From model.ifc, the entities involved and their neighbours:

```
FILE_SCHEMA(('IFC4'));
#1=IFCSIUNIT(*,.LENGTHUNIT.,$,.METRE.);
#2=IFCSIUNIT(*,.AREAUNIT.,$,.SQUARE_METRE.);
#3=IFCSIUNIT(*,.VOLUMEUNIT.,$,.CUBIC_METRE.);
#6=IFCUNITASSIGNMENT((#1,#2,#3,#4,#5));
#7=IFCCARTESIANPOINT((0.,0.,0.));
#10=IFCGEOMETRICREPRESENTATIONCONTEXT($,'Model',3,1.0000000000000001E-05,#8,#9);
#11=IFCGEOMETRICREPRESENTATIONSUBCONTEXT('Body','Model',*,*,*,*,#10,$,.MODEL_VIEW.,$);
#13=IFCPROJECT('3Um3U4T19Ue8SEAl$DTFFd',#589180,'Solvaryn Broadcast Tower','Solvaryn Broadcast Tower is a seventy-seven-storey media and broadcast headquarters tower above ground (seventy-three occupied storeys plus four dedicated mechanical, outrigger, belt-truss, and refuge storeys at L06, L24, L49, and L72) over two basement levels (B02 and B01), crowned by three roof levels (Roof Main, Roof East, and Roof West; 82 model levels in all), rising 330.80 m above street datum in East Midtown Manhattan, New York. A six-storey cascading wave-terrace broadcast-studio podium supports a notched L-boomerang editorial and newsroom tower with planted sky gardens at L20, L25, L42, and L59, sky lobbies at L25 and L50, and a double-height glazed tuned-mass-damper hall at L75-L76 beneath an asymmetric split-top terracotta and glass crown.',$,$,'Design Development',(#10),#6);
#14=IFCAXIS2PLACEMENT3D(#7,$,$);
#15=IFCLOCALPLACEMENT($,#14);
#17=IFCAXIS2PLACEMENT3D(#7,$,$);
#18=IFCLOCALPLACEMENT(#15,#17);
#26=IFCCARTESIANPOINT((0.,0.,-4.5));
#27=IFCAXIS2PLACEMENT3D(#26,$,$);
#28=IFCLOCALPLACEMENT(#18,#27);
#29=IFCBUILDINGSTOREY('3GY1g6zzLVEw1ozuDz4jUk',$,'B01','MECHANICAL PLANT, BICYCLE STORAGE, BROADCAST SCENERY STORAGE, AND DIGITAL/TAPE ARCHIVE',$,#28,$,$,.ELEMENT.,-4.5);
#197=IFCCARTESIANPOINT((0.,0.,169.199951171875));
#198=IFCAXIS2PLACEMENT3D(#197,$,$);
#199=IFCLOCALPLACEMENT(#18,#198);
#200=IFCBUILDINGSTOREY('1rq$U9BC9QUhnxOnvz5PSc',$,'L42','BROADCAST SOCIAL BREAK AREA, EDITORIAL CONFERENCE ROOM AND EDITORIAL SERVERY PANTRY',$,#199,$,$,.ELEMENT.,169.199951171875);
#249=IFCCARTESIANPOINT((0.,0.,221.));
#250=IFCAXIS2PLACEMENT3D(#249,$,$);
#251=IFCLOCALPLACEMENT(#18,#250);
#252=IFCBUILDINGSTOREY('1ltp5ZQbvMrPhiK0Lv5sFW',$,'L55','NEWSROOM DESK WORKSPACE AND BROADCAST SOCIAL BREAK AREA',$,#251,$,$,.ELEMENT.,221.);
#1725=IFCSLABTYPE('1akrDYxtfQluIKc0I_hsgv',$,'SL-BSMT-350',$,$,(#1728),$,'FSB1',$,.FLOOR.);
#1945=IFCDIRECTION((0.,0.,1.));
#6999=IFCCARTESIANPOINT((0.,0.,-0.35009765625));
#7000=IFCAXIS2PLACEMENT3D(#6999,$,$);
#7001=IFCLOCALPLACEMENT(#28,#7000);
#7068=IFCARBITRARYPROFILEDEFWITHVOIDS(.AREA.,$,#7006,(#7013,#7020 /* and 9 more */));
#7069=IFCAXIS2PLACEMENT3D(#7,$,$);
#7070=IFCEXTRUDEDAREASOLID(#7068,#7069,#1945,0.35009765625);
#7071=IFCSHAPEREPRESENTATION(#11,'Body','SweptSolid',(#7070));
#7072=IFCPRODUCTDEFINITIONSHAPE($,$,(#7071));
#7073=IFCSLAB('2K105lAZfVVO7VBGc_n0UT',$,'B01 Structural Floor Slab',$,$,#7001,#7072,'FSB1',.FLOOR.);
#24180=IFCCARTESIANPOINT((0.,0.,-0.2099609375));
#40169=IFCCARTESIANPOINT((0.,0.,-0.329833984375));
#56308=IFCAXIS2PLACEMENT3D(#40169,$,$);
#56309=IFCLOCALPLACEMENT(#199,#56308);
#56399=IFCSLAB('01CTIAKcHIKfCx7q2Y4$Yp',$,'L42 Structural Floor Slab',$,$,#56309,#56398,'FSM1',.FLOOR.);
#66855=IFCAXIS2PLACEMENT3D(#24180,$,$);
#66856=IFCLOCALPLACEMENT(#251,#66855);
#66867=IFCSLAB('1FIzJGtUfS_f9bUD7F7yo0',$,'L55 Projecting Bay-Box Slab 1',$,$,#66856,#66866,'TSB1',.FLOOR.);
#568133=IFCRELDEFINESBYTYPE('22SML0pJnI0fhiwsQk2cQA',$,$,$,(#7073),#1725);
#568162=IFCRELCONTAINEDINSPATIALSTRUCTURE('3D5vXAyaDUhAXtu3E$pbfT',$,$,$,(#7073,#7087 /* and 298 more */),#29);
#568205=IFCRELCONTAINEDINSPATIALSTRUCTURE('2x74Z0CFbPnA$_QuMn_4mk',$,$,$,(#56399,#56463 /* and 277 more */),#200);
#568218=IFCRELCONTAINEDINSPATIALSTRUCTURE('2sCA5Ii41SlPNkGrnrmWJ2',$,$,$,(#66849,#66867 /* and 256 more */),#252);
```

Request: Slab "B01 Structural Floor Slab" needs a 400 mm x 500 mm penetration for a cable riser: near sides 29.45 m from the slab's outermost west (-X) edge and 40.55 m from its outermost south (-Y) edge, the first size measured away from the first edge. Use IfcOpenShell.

```python
import numpy as np
import ifcopenshell
import ifcopenshell.api.feature
import ifcopenshell.api.geometry
import ifcopenshell.api.root
import ifcopenshell.geom
import ifcopenshell.util.placement
import ifcopenshell.util.representation
import ifcopenshell.util.shape
import ifcopenshell.util.unit

model = ifcopenshell.open("model.ifc")
unit_scale = ifcopenshell.util.unit.calculate_unit_scale(model)
settings = ifcopenshell.geom.settings()


def volume(element):
    """Net volume in cubic metres, openings subtracted."""
    shape = ifcopenshell.geom.create_shape(settings, element)
    return ifcopenshell.util.shape.get_volume(shape.geometry)


slab = model.by_guid("2K105lAZfVVO7VBGc_n0UT")
before = volume(slab)

# Extent in the slab's own axes, in metres. The edges named are its -X and -Y sides.
slab_shape = ifcopenshell.geom.create_shape(settings, slab)
vertices = ifcopenshell.util.shape.get_vertices(slab_shape.geometry)
x_min, y_min, bottom = vertices.min(axis=0)
top = vertices[:, 2].max()

opening = ifcopenshell.api.root.create_entity(model, ifc_class="IfcOpeningElement", name="Cable riser opening", predefined_type="OPENING")
context = ifcopenshell.util.representation.get_context(model, "Model", "Body", "MODEL_VIEW")
width, depth = 0.4, 0.5
outline = [(0.0, 0.0), (width, 0.0), (width, depth), (0.0, depth), (0.0, 0.0)]
# Overshoot both faces by 50 mm so the cut is clean.
shape = ifcopenshell.api.geometry.add_slab_representation(
    model, context=context, depth=top - bottom + 0.1, polyline=outline
)
ifcopenshell.api.geometry.assign_representation(model, product=opening, representation=shape)

matrix = ifcopenshell.util.placement.get_local_placement(slab.ObjectPlacement)
matrix[:, 3] = matrix @ np.append(np.array([x_min + 29.45, y_min + 40.55, bottom - 0.05]) / unit_scale, 1.0)
ifcopenshell.api.geometry.edit_object_placement(model, product=opening, matrix=matrix, is_si=False)
ifcopenshell.api.feature.add_feature(model, feature=opening, element=slab)

after = volume(slab)

print(f"slab volume {before:.3f} -> {after:.3f} m3")

model.write("model_updated.ifc")
```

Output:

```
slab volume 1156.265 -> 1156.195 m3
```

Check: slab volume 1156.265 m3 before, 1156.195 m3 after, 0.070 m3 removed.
